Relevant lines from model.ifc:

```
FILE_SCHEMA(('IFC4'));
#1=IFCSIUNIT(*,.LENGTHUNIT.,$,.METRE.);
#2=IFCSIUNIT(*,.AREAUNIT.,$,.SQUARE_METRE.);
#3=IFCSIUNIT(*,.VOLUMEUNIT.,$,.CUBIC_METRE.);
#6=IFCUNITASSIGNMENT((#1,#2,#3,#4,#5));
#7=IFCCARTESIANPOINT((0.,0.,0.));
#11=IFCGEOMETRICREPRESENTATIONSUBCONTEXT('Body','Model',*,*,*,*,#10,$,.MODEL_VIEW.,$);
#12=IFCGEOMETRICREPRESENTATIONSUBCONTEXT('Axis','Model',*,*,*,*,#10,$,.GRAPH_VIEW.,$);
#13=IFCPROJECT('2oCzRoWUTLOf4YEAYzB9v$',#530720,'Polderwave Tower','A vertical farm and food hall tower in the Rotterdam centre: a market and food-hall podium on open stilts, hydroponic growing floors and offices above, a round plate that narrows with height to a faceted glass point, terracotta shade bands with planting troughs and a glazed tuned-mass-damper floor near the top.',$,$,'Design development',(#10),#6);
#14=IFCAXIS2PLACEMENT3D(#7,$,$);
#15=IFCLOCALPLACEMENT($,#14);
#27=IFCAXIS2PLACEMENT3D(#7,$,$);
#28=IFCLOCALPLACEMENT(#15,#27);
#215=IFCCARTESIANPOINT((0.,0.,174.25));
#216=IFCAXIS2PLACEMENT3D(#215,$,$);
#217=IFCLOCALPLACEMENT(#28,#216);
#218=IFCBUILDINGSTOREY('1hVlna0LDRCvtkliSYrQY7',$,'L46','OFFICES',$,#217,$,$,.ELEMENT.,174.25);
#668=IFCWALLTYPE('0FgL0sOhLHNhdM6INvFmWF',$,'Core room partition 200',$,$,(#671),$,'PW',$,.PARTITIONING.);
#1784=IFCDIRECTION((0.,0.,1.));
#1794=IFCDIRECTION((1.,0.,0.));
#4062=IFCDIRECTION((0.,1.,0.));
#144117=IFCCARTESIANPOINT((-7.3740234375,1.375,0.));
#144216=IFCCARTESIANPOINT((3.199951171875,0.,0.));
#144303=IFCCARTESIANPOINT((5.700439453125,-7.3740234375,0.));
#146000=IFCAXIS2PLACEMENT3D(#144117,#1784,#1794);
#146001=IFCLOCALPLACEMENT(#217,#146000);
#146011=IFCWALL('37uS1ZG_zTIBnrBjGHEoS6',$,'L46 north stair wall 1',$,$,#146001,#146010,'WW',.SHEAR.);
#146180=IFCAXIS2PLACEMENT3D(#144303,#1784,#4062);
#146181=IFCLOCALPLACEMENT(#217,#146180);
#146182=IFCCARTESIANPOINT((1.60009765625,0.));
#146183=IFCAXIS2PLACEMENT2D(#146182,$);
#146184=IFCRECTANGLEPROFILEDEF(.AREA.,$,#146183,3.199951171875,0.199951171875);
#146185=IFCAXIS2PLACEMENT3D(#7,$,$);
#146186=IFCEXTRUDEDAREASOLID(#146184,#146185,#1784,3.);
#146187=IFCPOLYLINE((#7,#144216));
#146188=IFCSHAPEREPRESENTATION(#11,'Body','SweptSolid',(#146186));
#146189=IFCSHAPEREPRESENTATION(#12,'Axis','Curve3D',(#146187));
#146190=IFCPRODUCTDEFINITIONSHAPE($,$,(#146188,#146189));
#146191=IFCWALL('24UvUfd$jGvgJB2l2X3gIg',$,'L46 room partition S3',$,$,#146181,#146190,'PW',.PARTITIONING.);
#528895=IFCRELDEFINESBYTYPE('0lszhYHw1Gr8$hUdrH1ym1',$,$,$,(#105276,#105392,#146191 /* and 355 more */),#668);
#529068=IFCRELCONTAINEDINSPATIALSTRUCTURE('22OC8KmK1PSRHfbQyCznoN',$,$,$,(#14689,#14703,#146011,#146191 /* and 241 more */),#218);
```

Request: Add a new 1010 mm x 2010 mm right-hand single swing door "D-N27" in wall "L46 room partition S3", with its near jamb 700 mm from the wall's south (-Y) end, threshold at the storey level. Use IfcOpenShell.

```python
import numpy as np
import ifcopenshell
import ifcopenshell.api.feature
import ifcopenshell.api.geometry
import ifcopenshell.api.root
import ifcopenshell.api.spatial
import ifcopenshell.geom
import ifcopenshell.util.element
import ifcopenshell.util.placement
import ifcopenshell.util.representation
import ifcopenshell.util.shape
import ifcopenshell.util.unit

model = ifcopenshell.open("model.ifc")
unit_scale = ifcopenshell.util.unit.calculate_unit_scale(model)
settings = ifcopenshell.geom.settings()


def volume(element):
    """Net volume in cubic metres, openings subtracted."""
    shape = ifcopenshell.geom.create_shape(settings, element)
    return ifcopenshell.util.shape.get_volume(shape.geometry)


wall = model.by_guid("24UvUfd$jGvgJB2l2X3gIg")
storey = ifcopenshell.util.element.get_container(wall, ifc_class="IfcBuildingStorey")
context = ifcopenshell.util.representation.get_context(model, "Model", "Body", "MODEL_VIEW")
before = volume(wall)

width, height, from_end, sill = 1.01, 2.01, 0.7, 0.0  # metres

# The wall runs along its own X axis, and the end named is its -X end.
wall_shape = ifcopenshell.geom.create_shape(settings, wall)
x, y, z = ifcopenshell.util.shape.get_vertices(wall_shape.geometry).T
start = x.min() + from_end
face, thickness = float(y.min()), float(y.max() - y.min())
wall_matrix = ifcopenshell.util.placement.get_local_placement(wall.ObjectPlacement)
level = ifcopenshell.util.placement.get_local_placement(storey.ObjectPlacement)[2, 3]


def in_wall(x, y):
    """Placement at x, y metres in the wall's axes, at sill height."""
    matrix = wall_matrix.copy()
    matrix[:, 3] = wall_matrix @ np.array([x / unit_scale, y / unit_scale, 0.0, 1.0])
    matrix[2, 3] = level + sill / unit_scale
    return matrix


# Opening: a box that overshoots both wall faces by 50 mm.
opening = ifcopenshell.api.root.create_entity(model, ifc_class="IfcOpeningElement", predefined_type="OPENING")
box = ifcopenshell.api.geometry.add_wall_representation(
    model, context=context, length=width, height=height, thickness=thickness + 0.1
)
ifcopenshell.api.geometry.assign_representation(model, product=opening, representation=box)
ifcopenshell.api.geometry.edit_object_placement(model, product=opening, matrix=in_wall(start, face - 0.05), is_si=False)
ifcopenshell.api.feature.add_feature(model, feature=opening, element=wall)

door = ifcopenshell.api.root.create_entity(model, ifc_class="IfcDoor", name="D-N27", predefined_type="DOOR")
door.OverallWidth, door.OverallHeight = width / unit_scale, height / unit_scale
door.OperationType = "SINGLE_SWING_RIGHT"
body = ifcopenshell.api.geometry.add_door_representation(
    model,
    context=context,
    overall_width=door.OverallWidth,
    overall_height=door.OverallHeight,
    operation_type="SINGLE_SWING_RIGHT",
    lining_properties={"LiningDepth": thickness / unit_scale, "ThresholdDepth": thickness / unit_scale},
)
ifcopenshell.api.geometry.assign_representation(model, product=door, representation=body)
ifcopenshell.api.spatial.assign_container(model, products=[door], relating_structure=storey)
ifcopenshell.api.feature.add_filling(model, opening=opening, element=door)

# The lining spans the wall, so the door starts at the wall face.
ifcopenshell.api.geometry.edit_object_placement(model, product=door, matrix=in_wall(start, face), is_si=False)

after = volume(wall)

print(f"wall volume {before:.3f} -> {after:.3f} m3")

model.write("model_edited.ifc")
```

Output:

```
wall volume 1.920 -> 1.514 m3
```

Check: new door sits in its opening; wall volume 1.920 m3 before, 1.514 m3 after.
